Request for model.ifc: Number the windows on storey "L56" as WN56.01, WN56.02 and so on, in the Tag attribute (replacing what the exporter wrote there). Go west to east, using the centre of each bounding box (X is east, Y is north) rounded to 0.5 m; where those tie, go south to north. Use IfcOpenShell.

First a look at what the model holds.

```python
import ifcopenshell
import ifcopenshell.util.element
import ifcopenshell.util.placement

model = ifcopenshell.open("model.ifc")
print(model.schema)
storey = next(s for s in model.by_type("IfcBuildingStorey") if s.Name == "L56")
windows = [e for e in ifcopenshell.util.element.get_decomposition(storey) if e.is_a("IfcWindow")]
for e in sorted(windows, key=lambda e: e.id()):
    origin = ifcopenshell.util.placement.get_local_placement(e.ObjectPlacement)[:3, 3]
    print(e.id(), e.Tag, e.Name, origin.round(2) + 0.0, sep=" | ")
```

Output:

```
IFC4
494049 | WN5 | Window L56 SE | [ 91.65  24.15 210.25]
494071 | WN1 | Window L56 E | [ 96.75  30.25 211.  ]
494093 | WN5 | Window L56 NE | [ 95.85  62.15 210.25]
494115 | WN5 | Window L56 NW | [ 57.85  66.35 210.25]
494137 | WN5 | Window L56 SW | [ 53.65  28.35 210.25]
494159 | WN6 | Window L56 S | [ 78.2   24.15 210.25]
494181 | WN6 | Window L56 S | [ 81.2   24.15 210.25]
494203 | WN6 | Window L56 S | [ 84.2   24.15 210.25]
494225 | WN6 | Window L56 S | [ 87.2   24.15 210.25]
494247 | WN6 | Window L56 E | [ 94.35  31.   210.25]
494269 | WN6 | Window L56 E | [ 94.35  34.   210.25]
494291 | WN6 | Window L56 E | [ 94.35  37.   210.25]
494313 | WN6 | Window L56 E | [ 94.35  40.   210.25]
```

```python
import ifcopenshell
import ifcopenshell.geom
import ifcopenshell.util.element
import ifcopenshell.util.shape

model = ifcopenshell.open("model.ifc")
settings = ifcopenshell.geom.settings()
settings.set("use-world-coords", True)


def centre(element):
    shape = ifcopenshell.geom.create_shape(settings, element)
    return ifcopenshell.util.shape.get_bbox_centroid(shape.geometry)


storey = next(s for s in model.by_type("IfcBuildingStorey") if s.Name == "L56")
windows = [e for e in ifcopenshell.util.element.get_decomposition(storey) if e.is_a("IfcWindow")]

# Insertion points can sit at a corner or the storey origin, so sort by the geometry (in metres).
centres = {e: centre(e) for e in windows}
windows.sort(key=lambda e: (round(centres[e][0] / 0.5), centres[e][1]))

for i, e in enumerate(windows, start=1):
    number = f"WN56.{i:02d}"
    e.Tag = number
    print(e.id(), number)

model.write("model_rev.ifc")
```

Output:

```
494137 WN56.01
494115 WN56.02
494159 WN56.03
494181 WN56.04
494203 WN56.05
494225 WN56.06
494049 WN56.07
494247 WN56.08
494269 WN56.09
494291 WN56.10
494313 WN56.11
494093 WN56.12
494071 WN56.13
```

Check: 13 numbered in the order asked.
